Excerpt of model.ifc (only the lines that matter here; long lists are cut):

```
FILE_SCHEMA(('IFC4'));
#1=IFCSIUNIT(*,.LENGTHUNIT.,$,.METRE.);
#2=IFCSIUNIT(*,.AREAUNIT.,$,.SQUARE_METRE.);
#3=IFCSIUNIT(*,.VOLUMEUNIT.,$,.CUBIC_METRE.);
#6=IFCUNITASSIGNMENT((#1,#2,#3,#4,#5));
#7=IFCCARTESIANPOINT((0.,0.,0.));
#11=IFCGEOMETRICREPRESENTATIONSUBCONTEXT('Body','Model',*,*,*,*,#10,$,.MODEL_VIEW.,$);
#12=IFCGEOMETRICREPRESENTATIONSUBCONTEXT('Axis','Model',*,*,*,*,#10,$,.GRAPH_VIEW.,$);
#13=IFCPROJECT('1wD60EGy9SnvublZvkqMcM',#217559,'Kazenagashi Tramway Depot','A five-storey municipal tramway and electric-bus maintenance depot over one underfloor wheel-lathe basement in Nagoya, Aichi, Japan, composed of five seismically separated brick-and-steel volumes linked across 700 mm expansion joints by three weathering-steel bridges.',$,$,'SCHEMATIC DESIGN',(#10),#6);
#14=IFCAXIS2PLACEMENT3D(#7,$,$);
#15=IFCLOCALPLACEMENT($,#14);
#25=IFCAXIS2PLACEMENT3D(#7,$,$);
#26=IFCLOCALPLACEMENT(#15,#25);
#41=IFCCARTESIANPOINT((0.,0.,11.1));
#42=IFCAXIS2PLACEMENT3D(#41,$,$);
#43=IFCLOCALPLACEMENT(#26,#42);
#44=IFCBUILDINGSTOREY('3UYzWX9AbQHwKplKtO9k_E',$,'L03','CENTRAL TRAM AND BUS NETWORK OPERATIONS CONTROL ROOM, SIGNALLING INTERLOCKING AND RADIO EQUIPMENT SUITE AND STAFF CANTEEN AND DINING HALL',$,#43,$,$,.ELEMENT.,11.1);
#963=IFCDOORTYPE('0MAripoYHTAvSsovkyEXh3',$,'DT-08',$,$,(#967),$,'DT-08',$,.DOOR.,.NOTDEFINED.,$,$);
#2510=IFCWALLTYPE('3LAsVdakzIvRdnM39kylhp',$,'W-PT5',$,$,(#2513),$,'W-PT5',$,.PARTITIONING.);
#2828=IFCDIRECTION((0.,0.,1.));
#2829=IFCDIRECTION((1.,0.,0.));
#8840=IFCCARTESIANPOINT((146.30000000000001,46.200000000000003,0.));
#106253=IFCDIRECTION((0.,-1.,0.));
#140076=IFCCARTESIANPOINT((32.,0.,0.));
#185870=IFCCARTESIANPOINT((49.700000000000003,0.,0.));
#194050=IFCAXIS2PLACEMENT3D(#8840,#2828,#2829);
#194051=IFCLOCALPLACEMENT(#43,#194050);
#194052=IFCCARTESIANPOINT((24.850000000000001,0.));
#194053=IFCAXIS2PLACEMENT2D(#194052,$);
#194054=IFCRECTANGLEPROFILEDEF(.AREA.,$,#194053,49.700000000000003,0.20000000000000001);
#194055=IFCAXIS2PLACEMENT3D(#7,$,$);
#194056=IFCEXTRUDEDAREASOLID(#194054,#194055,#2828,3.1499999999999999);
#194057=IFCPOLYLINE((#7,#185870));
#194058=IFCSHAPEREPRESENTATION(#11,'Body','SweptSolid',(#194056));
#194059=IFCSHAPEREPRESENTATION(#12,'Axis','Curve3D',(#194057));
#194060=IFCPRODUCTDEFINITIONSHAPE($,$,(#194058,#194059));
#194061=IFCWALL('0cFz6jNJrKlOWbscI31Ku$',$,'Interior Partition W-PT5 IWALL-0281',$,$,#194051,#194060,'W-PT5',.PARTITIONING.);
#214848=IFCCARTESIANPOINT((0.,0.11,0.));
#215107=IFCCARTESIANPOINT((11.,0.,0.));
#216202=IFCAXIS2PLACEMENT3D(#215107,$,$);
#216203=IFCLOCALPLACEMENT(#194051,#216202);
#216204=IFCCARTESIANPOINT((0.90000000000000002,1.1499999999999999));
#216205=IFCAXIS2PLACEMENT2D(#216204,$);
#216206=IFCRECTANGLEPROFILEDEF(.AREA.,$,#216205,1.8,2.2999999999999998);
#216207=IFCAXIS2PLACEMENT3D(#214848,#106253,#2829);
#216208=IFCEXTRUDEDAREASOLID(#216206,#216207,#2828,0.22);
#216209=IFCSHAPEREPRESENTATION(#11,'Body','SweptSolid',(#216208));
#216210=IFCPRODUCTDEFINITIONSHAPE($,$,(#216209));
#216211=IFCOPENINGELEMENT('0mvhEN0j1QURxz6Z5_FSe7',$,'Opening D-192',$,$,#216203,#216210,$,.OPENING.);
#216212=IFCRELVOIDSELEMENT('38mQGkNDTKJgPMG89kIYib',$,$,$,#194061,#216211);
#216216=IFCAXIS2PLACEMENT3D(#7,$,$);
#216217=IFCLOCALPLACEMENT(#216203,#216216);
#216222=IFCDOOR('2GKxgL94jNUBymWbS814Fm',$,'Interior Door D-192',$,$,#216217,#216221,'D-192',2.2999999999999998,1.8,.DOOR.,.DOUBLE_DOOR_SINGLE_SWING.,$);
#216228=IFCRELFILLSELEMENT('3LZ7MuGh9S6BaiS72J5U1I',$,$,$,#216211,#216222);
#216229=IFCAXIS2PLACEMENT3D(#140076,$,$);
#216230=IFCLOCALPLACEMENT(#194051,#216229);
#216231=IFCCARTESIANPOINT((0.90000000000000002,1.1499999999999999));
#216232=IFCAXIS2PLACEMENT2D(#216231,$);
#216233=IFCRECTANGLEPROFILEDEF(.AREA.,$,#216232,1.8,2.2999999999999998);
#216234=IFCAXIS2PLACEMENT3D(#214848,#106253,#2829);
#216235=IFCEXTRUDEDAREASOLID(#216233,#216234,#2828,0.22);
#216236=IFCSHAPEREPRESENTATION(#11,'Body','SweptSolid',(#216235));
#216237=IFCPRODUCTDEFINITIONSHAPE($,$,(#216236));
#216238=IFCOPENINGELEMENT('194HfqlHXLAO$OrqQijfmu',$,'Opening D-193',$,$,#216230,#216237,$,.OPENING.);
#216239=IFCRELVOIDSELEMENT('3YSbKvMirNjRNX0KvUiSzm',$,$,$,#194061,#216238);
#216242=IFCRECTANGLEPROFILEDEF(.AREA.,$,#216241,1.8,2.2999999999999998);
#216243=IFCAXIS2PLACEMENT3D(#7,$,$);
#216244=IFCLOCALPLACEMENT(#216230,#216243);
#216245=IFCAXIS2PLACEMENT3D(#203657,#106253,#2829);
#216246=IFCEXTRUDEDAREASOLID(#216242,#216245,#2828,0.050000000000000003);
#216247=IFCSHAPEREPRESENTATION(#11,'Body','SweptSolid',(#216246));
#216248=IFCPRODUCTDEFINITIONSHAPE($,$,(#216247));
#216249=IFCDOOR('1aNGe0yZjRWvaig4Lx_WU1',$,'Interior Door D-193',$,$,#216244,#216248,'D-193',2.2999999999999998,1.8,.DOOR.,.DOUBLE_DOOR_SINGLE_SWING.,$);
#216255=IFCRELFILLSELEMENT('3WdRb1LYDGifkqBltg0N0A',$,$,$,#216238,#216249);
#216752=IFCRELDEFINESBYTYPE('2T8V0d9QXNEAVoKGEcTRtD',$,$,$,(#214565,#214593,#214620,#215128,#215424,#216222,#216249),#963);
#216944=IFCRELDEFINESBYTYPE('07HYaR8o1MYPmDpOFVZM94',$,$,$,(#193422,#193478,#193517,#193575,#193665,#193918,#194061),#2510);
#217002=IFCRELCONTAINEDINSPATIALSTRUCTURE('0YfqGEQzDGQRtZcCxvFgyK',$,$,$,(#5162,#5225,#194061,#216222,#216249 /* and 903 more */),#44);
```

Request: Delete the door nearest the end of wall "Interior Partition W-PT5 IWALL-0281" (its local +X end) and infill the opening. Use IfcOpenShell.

```python
import ifcopenshell
import ifcopenshell.api.feature
import ifcopenshell.api.root
import ifcopenshell.geom
import ifcopenshell.util.shape

model = ifcopenshell.open("model.ifc")
settings = ifcopenshell.geom.settings()


def volume(element):
    """Net volume in cubic metres, openings subtracted."""
    shape = ifcopenshell.geom.create_shape(settings, element)
    return ifcopenshell.util.shape.get_volume(shape.geometry)


door = model.by_guid("1aNGe0yZjRWvaig4Lx_WU1")
opening = door.FillsVoids[0].RelatingOpeningElement
wall = opening.VoidsElements[0].RelatingBuildingElement
before = volume(wall)

ifcopenshell.api.root.remove_product(model, product=door)
ifcopenshell.api.feature.remove_feature(model, feature=opening)

after = volume(wall)

print(f"wall volume {before:.3f} -> {after:.3f} m3")

model.write("model_v2.ifc")
```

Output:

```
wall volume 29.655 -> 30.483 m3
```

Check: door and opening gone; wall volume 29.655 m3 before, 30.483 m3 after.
